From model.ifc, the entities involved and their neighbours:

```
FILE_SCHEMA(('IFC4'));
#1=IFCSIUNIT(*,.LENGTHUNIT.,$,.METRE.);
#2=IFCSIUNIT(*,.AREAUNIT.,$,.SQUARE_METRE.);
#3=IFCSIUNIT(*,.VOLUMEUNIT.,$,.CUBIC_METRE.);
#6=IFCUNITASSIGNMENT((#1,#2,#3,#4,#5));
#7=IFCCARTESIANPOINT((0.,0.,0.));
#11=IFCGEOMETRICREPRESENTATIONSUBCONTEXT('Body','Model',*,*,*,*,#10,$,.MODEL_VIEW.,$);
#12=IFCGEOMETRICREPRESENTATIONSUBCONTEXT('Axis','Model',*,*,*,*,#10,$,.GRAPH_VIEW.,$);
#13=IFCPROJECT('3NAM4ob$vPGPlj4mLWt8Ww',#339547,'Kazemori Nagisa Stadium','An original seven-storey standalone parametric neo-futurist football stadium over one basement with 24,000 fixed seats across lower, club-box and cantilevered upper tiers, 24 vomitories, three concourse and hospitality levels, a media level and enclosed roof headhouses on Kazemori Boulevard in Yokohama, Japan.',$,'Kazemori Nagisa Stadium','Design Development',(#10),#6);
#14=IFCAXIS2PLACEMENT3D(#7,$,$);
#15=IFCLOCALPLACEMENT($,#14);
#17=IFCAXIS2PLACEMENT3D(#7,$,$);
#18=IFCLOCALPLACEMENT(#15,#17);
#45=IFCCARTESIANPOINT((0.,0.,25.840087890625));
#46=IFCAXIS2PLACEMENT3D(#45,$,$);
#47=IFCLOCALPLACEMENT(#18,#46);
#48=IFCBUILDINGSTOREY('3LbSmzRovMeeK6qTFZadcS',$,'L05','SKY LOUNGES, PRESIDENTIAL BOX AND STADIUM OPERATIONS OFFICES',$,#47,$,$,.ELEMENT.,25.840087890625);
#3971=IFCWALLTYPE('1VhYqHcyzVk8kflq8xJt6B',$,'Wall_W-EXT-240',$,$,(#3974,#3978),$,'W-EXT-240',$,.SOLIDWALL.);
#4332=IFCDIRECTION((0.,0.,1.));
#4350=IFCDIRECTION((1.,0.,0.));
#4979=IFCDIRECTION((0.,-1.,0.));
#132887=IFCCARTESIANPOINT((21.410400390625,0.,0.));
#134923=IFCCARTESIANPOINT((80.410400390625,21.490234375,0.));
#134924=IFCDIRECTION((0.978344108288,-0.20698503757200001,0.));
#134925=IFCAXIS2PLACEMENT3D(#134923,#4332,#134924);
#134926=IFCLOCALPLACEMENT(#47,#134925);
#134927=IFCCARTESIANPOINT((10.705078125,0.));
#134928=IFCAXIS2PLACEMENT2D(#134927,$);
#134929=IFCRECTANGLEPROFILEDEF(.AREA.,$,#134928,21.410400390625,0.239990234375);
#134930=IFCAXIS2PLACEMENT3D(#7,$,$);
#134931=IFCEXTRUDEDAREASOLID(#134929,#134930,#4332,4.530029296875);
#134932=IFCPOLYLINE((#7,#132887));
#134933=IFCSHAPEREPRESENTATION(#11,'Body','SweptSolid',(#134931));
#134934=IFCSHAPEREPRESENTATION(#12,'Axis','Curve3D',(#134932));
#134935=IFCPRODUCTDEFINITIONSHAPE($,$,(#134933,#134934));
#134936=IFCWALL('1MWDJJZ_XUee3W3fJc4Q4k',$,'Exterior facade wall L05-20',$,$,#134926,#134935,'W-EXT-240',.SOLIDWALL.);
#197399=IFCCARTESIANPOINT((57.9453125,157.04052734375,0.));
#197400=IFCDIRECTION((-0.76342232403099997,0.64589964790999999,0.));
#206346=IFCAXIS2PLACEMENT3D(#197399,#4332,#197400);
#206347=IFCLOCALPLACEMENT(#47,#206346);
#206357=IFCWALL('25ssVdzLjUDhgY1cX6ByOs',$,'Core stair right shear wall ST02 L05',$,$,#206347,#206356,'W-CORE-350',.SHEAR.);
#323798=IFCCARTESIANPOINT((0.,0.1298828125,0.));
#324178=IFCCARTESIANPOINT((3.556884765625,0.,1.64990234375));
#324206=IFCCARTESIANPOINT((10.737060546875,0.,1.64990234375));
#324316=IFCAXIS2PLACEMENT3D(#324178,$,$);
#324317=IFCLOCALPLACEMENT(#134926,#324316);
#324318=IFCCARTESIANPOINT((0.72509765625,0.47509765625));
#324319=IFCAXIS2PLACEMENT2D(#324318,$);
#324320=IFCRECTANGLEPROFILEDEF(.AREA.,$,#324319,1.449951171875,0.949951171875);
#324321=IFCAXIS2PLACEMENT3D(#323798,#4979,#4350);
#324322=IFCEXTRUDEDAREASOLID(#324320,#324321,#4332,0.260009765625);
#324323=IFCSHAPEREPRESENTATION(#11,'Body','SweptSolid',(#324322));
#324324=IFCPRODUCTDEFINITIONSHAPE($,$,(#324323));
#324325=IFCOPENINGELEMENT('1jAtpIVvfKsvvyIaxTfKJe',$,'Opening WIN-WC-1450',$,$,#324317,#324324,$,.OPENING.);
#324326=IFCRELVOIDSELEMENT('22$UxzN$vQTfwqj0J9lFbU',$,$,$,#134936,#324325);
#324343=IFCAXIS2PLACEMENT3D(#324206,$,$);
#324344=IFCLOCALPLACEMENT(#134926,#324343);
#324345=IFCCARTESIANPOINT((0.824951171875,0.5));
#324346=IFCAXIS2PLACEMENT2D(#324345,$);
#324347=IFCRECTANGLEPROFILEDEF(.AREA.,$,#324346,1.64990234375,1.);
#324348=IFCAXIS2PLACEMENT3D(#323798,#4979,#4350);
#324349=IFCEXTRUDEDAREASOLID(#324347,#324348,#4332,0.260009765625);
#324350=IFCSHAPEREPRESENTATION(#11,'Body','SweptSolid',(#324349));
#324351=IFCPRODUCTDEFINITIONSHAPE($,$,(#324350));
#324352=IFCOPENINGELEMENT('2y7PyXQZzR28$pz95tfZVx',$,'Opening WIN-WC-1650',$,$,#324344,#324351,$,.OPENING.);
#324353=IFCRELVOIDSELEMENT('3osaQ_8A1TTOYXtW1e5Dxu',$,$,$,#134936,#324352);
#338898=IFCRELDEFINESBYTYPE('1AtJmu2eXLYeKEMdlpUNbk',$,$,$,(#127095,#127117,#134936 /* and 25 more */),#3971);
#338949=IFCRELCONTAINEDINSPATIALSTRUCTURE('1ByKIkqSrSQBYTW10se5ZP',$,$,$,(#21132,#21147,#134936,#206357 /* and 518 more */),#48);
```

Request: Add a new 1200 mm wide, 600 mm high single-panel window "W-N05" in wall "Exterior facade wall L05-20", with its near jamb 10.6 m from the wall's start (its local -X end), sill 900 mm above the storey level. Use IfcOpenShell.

```python
import numpy as np
import ifcopenshell
import ifcopenshell.api.feature
import ifcopenshell.api.geometry
import ifcopenshell.api.root
import ifcopenshell.api.spatial
import ifcopenshell.geom
import ifcopenshell.util.element
import ifcopenshell.util.placement
import ifcopenshell.util.representation
import ifcopenshell.util.shape
import ifcopenshell.util.unit

model = ifcopenshell.open("model.ifc")
unit_scale = ifcopenshell.util.unit.calculate_unit_scale(model)
settings = ifcopenshell.geom.settings()


def volume(element):
    """Net volume in cubic metres, openings subtracted."""
    shape = ifcopenshell.geom.create_shape(settings, element)
    return ifcopenshell.util.shape.get_volume(shape.geometry)


wall = model.by_guid("1MWDJJZ_XUee3W3fJc4Q4k")
storey = ifcopenshell.util.element.get_container(wall, ifc_class="IfcBuildingStorey")
context = ifcopenshell.util.representation.get_context(model, "Model", "Body", "MODEL_VIEW")
before = volume(wall)

width, height, from_end, sill = 1.2, 0.6, 10.6, 0.9  # metres

# The wall runs along its own X axis, and the end named is its -X end.
wall_shape = ifcopenshell.geom.create_shape(settings, wall)
x, y, z = ifcopenshell.util.shape.get_vertices(wall_shape.geometry).T
start = x.min() + from_end
face, thickness = float(y.min()), float(y.max() - y.min())
wall_matrix = ifcopenshell.util.placement.get_local_placement(wall.ObjectPlacement)
level = ifcopenshell.util.placement.get_local_placement(storey.ObjectPlacement)[2, 3]


def in_wall(x, y):
    """Placement at x, y metres in the wall's axes, at sill height."""
    matrix = wall_matrix.copy()
    matrix[:, 3] = wall_matrix @ np.array([x / unit_scale, y / unit_scale, 0.0, 1.0])
    matrix[2, 3] = level + sill / unit_scale
    return matrix


# Opening: a box that overshoots both wall faces by 50 mm.
opening = ifcopenshell.api.root.create_entity(model, ifc_class="IfcOpeningElement", predefined_type="OPENING")
box = ifcopenshell.api.geometry.add_wall_representation(
    model, context=context, length=width, height=height, thickness=thickness + 0.1
)
ifcopenshell.api.geometry.assign_representation(model, product=opening, representation=box)
ifcopenshell.api.geometry.edit_object_placement(model, product=opening, matrix=in_wall(start, face - 0.05), is_si=False)
ifcopenshell.api.feature.add_feature(model, feature=opening, element=wall)

window = ifcopenshell.api.root.create_entity(model, ifc_class="IfcWindow", name="W-N05", predefined_type="WINDOW")
window.OverallWidth, window.OverallHeight = width / unit_scale, height / unit_scale
window.PartitioningType = "SINGLE_PANEL"
body = ifcopenshell.api.geometry.add_window_representation(
    model,
    context=context,
    overall_width=window.OverallWidth,
    overall_height=window.OverallHeight,
    partition_type="SINGLE_PANEL",
)
ifcopenshell.api.geometry.assign_representation(model, product=window, representation=body)
ifcopenshell.api.spatial.assign_container(model, products=[window], relating_structure=storey)
ifcopenshell.api.feature.add_filling(model, opening=opening, element=window)

# Centre the window in the wall's thickness.
ifcopenshell.api.geometry.edit_object_placement(model, product=window, matrix=in_wall(start, face), is_si=False)
window_shape = ifcopenshell.geom.create_shape(settings, window)
depth = ifcopenshell.util.shape.get_vertices(window_shape.geometry)[:, 1]
offset = face + thickness / 2 - (depth.min() + depth.max()) / 2
ifcopenshell.api.geometry.edit_object_placement(model, product=window, matrix=in_wall(start, offset), is_si=False)

after = volume(wall)

print(f"wall volume {before:.3f} -> {after:.3f} m3")

model.write("model_v2.ifc")
```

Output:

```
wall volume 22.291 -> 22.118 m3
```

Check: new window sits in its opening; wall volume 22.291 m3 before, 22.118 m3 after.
